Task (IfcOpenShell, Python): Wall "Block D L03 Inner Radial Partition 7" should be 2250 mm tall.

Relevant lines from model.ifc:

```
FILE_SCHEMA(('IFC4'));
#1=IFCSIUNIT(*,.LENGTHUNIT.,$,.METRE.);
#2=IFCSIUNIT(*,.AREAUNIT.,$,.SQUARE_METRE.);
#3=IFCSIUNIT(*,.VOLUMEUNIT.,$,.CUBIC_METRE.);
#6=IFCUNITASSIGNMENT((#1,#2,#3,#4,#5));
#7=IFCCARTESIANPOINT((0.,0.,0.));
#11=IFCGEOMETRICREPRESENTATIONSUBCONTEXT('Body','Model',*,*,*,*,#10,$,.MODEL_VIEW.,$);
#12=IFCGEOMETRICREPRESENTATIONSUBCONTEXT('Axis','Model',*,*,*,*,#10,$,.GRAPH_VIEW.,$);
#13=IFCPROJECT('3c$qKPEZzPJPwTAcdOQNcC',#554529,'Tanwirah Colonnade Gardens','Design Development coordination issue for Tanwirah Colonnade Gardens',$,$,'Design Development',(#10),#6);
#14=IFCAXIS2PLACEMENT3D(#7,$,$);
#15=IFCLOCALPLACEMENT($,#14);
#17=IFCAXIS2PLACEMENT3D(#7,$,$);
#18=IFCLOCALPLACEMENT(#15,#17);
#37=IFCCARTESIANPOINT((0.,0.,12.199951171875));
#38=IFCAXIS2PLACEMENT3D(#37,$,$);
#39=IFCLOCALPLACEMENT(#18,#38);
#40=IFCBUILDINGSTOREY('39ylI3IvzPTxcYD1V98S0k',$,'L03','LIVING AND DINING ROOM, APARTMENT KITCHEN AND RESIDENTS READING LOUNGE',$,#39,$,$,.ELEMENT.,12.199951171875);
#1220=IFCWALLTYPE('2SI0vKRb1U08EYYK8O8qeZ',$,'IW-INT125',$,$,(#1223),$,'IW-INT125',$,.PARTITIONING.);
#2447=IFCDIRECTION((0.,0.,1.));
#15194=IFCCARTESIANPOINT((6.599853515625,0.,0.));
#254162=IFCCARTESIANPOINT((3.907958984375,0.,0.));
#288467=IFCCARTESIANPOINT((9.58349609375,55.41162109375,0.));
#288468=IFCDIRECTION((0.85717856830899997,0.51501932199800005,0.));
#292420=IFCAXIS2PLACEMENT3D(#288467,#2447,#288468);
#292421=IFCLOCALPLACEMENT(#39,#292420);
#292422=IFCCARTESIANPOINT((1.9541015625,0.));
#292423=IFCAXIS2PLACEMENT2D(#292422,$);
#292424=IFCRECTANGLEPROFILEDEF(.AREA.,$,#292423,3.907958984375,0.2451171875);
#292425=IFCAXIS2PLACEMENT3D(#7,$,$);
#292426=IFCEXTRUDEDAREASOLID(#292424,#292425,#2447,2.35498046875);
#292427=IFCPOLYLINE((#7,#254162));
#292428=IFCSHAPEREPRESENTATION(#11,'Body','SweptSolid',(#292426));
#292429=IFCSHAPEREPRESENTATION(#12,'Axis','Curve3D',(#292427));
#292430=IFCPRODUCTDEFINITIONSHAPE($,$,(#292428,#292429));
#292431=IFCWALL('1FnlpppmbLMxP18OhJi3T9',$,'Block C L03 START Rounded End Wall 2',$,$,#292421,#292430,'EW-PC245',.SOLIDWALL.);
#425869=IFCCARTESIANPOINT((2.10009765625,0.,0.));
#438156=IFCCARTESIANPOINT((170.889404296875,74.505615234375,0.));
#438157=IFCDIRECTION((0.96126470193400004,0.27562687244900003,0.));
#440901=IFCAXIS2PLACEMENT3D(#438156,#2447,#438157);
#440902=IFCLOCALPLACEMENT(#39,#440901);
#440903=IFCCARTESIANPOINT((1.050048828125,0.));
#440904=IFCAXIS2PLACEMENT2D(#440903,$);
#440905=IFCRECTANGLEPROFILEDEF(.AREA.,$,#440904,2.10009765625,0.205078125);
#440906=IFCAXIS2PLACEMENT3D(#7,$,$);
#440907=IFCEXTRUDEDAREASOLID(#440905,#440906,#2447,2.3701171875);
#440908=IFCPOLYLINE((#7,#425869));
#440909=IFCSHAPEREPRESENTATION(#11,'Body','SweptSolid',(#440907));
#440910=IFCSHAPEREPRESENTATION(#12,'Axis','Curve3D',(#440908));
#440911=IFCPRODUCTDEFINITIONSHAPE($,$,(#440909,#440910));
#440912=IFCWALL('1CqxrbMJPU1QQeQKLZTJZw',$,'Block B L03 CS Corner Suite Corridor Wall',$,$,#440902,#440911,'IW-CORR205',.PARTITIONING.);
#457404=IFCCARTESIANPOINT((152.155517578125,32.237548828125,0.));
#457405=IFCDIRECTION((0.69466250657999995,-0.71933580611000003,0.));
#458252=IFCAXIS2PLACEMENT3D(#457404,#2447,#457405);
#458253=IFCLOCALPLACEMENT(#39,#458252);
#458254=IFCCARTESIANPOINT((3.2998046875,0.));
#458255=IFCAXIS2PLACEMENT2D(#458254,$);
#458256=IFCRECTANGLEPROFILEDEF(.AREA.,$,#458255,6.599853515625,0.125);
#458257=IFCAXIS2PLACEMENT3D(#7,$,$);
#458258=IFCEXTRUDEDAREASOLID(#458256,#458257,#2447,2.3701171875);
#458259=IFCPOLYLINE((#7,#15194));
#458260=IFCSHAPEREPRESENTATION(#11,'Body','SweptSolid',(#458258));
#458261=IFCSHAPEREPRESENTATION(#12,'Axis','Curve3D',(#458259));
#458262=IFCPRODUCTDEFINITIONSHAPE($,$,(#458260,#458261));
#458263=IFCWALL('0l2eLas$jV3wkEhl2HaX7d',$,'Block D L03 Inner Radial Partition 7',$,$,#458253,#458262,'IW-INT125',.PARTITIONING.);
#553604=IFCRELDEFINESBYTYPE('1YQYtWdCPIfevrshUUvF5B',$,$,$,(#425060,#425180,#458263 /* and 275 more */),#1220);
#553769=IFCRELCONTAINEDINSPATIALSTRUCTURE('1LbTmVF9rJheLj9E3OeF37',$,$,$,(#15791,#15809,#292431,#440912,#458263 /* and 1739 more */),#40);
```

```python
import ifcopenshell
import ifcopenshell.geom
import ifcopenshell.util.representation
import ifcopenshell.util.shape

model = ifcopenshell.open("model.ifc")
settings = ifcopenshell.geom.settings()


def volume(element):
    """Net volume in cubic metres, openings subtracted."""
    shape = ifcopenshell.geom.create_shape(settings, element)
    return ifcopenshell.util.shape.get_volume(shape.geometry)


wall = model.by_guid("0l2eLas$jV3wkEhl2HaX7d")
before = volume(wall)

body = ifcopenshell.util.representation.get_representation(wall, "Model", "Body")
solid = body.Items[0]
old_height = solid.Depth
solid.Depth = 2.25
after = volume(wall)

print(f"height {old_height:g} -> {solid.Depth:g}, volume {before:.3f} -> {after:.3f} m3")

model.write("model_v2.ifc")
```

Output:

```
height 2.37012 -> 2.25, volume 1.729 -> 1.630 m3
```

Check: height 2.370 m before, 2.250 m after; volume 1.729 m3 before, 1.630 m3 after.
